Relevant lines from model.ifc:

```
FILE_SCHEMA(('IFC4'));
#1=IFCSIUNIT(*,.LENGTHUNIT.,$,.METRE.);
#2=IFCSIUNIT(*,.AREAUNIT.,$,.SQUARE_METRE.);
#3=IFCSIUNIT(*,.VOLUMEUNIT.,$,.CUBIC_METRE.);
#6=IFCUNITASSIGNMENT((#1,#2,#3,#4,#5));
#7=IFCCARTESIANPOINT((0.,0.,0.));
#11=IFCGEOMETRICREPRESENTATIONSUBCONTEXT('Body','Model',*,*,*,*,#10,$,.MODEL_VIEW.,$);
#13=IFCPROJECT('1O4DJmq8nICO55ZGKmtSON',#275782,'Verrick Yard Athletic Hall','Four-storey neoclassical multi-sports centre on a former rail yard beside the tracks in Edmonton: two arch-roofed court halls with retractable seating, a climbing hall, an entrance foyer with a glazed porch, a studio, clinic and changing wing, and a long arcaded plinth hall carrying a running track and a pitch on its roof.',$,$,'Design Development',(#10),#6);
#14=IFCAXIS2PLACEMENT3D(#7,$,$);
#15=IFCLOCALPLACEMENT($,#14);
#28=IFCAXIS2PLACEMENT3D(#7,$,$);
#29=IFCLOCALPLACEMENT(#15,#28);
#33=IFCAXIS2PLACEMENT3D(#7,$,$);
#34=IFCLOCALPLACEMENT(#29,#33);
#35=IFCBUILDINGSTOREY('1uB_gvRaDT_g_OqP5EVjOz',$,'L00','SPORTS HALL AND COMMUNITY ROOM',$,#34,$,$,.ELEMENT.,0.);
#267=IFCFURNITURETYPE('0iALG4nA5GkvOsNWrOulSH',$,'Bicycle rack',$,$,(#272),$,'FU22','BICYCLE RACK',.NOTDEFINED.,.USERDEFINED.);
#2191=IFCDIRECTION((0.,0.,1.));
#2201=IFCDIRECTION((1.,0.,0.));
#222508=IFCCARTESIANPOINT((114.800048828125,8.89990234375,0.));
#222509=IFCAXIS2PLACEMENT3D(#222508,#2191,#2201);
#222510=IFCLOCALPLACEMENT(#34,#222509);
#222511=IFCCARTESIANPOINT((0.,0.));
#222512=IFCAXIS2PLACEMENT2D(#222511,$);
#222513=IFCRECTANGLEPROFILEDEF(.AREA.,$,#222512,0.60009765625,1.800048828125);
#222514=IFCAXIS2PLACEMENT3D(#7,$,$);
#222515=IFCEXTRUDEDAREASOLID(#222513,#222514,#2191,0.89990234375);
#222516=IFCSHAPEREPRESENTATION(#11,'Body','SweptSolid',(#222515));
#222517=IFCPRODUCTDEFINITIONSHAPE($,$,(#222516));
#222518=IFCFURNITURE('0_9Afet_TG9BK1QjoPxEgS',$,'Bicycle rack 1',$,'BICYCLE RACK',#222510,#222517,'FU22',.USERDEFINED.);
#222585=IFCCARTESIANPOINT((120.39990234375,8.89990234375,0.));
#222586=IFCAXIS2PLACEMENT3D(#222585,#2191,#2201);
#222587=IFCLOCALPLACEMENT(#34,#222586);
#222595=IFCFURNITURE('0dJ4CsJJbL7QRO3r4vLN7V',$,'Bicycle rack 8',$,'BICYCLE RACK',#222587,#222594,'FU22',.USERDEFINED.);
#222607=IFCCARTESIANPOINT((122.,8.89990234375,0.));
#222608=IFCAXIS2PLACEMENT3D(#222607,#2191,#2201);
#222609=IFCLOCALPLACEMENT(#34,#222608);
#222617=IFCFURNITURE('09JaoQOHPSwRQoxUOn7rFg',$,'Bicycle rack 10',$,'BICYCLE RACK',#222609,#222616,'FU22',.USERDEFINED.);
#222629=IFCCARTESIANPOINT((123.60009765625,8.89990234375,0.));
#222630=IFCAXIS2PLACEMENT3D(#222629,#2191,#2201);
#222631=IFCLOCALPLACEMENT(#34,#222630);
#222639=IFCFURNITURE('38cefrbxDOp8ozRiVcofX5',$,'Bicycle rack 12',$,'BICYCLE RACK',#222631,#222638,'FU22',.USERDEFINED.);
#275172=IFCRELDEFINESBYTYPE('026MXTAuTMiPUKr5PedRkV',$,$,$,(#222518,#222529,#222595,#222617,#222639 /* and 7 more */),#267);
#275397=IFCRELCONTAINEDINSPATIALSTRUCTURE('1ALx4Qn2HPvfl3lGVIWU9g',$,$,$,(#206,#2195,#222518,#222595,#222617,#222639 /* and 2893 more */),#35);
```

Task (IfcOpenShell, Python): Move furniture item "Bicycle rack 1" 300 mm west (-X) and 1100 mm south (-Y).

```python
import ifcopenshell
import ifcopenshell.api.geometry
import ifcopenshell.util.placement

model = ifcopenshell.open("model.ifc")

item = model.by_id(222518)
matrix = ifcopenshell.util.placement.get_local_placement(item.ObjectPlacement)
matrix[0, 3] -= 0.3
matrix[1, 3] -= 1.1
ifcopenshell.api.geometry.edit_object_placement(model, product=item, matrix=matrix, is_si=False)

print(ifcopenshell.util.placement.get_local_placement(item.ObjectPlacement).round(3) + 0.0)

model.write("model_updated.ifc")
```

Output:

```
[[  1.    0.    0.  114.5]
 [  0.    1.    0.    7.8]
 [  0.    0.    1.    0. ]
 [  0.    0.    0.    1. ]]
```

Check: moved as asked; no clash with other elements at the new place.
